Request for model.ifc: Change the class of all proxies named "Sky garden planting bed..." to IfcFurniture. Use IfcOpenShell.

First a look at what the model holds.

```python
import re

import ifcopenshell

model = ifcopenshell.open("model.ifc")
print(model.schema)
seen = {}
for e in model.by_type("IfcBuildingElementProxy"):
    name = re.sub(r":\d+(:\d+)?$", "", e.Name or "")  # drop the element id that some exporters append
    seen[name] = seen.get(name, 0) + 1
for name, count in sorted(seen.items()):
    print(count, "x", name)
```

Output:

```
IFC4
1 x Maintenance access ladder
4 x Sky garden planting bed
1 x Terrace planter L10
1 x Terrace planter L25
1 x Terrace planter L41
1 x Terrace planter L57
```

```python
import ifcopenshell
import ifcopenshell.api.root

model = ifcopenshell.open("model.ifc")

proxies = [e.id() for e in model.by_type("IfcBuildingElementProxy") if (e.Name or "").startswith("Sky garden planting bed")]
for step_id in proxies:
    proxy = model.by_id(step_id)
    ifcopenshell.api.root.reassign_class(model, product=proxy, ifc_class="IfcFurniture")

print(sum(model.by_id(i).is_a("IfcFurniture") for i in proxies), "reclassified")

model.write("model_rev.ifc")
```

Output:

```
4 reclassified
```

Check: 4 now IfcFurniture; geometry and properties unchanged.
